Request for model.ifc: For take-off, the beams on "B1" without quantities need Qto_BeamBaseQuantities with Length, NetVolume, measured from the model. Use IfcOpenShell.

First a look at what the model holds.

```python
import ifcopenshell
import ifcopenshell.util.element
import ifcopenshell.util.unit

model = ifcopenshell.open("model.ifc")
print(model.schema)
for unit_type in ("LENGTHUNIT", "AREAUNIT", "VOLUMEUNIT"):
    print(unit_type, ifcopenshell.util.unit.calculate_unit_scale(model, unit_type))
storey = next(s for s in model.by_type("IfcBuildingStorey") if s.Name == "B1")
beams = [e for e in ifcopenshell.util.element.get_decomposition(storey) if e.is_a("IfcBeam")]
for e in sorted(beams, key=lambda e: e.id()):
    print(e.id(), e.is_a(), e.Name, list(ifcopenshell.util.element.get_psets(e, qtos_only=True)), sep=" | ")
```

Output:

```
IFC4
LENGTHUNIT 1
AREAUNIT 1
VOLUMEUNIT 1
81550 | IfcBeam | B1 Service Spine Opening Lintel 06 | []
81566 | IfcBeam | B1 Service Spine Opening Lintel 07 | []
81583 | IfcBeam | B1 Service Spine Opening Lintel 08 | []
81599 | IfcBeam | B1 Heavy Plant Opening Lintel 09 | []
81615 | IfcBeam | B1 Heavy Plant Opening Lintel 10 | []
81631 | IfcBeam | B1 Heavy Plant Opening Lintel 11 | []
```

```python
import ifcopenshell
import ifcopenshell.api.pset
import ifcopenshell.geom
import ifcopenshell.util.element
import ifcopenshell.util.shape
import ifcopenshell.util.unit

model = ifcopenshell.open("model.ifc")
unit_scale = ifcopenshell.util.unit.calculate_unit_scale(model)
volume_scale = ifcopenshell.util.unit.calculate_unit_scale(model, "VOLUMEUNIT")
settings = ifcopenshell.geom.settings()

storey = next(s for s in model.by_type("IfcBuildingStorey") if s.Name == "B1")
beams = [e for e in ifcopenshell.util.element.get_decomposition(storey) if e.is_a("IfcBeam")]

for e in sorted(beams, key=lambda e: e.id()):
    if ifcopenshell.util.element.get_psets(e, qtos_only=True, should_inherit=False):
        continue
    # Geometry comes back in metres, in the element's own axes.
    shape = ifcopenshell.geom.create_shape(settings, e)
    values = {
        "Length": ifcopenshell.util.shape.get_max_xyz(shape.geometry) / unit_scale,
        "NetVolume": ifcopenshell.util.shape.get_volume(shape.geometry) / volume_scale,
    }
    qto = ifcopenshell.api.pset.add_qto(model, product=e, name="Qto_BeamBaseQuantities")
    ifcopenshell.api.pset.edit_qto(model, qto=qto, properties=values)
    print(e.id(), {k: round(v, 3) for k, v in values.items()})

model.write("model_edited.ifc")
```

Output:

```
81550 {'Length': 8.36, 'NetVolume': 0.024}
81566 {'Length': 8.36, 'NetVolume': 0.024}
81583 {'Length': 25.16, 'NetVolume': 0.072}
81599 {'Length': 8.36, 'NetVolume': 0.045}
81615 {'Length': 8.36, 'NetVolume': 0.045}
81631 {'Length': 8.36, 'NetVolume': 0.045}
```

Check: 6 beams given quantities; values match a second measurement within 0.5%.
